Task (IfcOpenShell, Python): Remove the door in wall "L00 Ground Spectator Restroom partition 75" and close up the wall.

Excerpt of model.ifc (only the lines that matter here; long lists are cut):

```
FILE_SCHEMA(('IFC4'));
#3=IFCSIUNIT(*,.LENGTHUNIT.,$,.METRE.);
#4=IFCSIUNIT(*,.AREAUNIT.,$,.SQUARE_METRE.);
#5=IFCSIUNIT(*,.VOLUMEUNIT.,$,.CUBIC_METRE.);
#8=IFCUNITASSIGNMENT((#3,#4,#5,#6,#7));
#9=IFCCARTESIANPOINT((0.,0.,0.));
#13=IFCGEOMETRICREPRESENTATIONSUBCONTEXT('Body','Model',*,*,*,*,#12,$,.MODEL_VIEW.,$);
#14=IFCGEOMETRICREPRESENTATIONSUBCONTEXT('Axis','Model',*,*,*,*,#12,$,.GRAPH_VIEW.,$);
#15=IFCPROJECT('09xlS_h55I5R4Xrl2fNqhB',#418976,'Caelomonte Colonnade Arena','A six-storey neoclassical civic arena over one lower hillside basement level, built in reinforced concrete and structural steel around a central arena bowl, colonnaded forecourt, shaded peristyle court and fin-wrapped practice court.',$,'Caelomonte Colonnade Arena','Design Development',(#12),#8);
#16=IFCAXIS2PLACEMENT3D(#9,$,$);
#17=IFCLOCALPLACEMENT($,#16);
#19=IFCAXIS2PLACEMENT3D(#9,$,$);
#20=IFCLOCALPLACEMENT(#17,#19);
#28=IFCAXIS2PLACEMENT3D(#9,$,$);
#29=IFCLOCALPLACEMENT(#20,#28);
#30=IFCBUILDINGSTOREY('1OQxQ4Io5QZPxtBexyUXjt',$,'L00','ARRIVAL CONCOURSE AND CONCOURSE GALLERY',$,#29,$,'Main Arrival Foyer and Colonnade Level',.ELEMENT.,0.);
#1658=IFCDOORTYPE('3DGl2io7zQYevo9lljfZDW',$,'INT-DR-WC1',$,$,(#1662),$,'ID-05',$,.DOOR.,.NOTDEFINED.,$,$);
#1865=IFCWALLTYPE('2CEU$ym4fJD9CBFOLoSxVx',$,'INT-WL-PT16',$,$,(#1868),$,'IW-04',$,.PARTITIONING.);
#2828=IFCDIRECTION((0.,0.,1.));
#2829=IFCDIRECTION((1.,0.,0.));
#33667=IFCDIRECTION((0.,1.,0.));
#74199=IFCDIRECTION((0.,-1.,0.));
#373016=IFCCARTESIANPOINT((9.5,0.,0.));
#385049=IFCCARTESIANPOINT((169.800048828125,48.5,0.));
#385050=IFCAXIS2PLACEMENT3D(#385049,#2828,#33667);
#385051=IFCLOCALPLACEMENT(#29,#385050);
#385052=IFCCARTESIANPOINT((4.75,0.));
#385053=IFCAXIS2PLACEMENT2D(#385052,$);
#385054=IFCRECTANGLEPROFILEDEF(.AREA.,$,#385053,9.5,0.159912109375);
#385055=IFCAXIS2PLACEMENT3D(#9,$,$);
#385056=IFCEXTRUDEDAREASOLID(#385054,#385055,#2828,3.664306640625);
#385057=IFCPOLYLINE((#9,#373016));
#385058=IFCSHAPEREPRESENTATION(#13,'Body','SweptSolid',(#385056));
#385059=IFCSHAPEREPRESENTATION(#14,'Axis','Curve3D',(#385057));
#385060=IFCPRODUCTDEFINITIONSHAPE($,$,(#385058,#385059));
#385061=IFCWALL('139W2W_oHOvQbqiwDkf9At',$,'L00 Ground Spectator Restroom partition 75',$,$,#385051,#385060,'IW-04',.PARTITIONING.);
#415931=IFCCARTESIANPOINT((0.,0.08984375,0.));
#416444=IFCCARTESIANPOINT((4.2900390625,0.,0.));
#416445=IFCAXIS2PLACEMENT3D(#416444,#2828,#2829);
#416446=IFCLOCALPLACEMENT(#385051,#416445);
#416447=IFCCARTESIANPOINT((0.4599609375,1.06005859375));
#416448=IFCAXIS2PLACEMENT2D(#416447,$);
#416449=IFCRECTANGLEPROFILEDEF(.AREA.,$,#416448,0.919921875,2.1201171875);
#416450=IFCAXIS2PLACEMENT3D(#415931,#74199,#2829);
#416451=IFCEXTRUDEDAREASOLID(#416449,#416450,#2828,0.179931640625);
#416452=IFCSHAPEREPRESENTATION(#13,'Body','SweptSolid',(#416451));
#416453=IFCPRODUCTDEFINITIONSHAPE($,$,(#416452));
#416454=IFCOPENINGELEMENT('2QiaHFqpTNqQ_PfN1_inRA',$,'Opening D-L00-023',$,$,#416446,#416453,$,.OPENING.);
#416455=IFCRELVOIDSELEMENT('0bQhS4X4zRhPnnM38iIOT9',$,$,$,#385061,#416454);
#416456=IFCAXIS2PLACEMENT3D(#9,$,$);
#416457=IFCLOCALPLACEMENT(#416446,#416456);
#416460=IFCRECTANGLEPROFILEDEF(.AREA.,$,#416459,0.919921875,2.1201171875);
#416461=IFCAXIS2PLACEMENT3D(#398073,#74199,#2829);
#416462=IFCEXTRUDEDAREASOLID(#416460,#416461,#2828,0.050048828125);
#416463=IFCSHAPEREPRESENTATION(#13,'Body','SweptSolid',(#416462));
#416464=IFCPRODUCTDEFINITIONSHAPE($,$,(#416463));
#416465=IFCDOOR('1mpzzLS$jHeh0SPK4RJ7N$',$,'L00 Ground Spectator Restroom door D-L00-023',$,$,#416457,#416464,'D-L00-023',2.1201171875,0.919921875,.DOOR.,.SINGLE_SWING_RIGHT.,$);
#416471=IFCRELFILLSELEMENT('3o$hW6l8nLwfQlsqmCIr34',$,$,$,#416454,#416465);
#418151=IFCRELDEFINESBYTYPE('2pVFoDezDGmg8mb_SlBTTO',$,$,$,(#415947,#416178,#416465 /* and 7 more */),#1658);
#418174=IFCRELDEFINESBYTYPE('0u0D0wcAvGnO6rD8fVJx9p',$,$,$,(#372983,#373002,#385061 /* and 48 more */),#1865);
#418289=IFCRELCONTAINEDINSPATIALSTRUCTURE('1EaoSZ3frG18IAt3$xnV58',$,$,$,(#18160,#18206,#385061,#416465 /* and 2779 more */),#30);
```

```python
import ifcopenshell
import ifcopenshell.api.feature
import ifcopenshell.api.root
import ifcopenshell.geom
import ifcopenshell.util.shape

model = ifcopenshell.open("model.ifc")
settings = ifcopenshell.geom.settings()


def volume(element):
    """Net volume in cubic metres, openings subtracted."""
    shape = ifcopenshell.geom.create_shape(settings, element)
    return ifcopenshell.util.shape.get_volume(shape.geometry)


door = model.by_id(416465)
opening = door.FillsVoids[0].RelatingOpeningElement
wall = opening.VoidsElements[0].RelatingBuildingElement
before = volume(wall)

ifcopenshell.api.root.remove_product(model, product=door)
ifcopenshell.api.feature.remove_feature(model, feature=opening)

after = volume(wall)

print(f"wall volume {before:.3f} -> {after:.3f} m3")

model.write("model_edited.ifc")
```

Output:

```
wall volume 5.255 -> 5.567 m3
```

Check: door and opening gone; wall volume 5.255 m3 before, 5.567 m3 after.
